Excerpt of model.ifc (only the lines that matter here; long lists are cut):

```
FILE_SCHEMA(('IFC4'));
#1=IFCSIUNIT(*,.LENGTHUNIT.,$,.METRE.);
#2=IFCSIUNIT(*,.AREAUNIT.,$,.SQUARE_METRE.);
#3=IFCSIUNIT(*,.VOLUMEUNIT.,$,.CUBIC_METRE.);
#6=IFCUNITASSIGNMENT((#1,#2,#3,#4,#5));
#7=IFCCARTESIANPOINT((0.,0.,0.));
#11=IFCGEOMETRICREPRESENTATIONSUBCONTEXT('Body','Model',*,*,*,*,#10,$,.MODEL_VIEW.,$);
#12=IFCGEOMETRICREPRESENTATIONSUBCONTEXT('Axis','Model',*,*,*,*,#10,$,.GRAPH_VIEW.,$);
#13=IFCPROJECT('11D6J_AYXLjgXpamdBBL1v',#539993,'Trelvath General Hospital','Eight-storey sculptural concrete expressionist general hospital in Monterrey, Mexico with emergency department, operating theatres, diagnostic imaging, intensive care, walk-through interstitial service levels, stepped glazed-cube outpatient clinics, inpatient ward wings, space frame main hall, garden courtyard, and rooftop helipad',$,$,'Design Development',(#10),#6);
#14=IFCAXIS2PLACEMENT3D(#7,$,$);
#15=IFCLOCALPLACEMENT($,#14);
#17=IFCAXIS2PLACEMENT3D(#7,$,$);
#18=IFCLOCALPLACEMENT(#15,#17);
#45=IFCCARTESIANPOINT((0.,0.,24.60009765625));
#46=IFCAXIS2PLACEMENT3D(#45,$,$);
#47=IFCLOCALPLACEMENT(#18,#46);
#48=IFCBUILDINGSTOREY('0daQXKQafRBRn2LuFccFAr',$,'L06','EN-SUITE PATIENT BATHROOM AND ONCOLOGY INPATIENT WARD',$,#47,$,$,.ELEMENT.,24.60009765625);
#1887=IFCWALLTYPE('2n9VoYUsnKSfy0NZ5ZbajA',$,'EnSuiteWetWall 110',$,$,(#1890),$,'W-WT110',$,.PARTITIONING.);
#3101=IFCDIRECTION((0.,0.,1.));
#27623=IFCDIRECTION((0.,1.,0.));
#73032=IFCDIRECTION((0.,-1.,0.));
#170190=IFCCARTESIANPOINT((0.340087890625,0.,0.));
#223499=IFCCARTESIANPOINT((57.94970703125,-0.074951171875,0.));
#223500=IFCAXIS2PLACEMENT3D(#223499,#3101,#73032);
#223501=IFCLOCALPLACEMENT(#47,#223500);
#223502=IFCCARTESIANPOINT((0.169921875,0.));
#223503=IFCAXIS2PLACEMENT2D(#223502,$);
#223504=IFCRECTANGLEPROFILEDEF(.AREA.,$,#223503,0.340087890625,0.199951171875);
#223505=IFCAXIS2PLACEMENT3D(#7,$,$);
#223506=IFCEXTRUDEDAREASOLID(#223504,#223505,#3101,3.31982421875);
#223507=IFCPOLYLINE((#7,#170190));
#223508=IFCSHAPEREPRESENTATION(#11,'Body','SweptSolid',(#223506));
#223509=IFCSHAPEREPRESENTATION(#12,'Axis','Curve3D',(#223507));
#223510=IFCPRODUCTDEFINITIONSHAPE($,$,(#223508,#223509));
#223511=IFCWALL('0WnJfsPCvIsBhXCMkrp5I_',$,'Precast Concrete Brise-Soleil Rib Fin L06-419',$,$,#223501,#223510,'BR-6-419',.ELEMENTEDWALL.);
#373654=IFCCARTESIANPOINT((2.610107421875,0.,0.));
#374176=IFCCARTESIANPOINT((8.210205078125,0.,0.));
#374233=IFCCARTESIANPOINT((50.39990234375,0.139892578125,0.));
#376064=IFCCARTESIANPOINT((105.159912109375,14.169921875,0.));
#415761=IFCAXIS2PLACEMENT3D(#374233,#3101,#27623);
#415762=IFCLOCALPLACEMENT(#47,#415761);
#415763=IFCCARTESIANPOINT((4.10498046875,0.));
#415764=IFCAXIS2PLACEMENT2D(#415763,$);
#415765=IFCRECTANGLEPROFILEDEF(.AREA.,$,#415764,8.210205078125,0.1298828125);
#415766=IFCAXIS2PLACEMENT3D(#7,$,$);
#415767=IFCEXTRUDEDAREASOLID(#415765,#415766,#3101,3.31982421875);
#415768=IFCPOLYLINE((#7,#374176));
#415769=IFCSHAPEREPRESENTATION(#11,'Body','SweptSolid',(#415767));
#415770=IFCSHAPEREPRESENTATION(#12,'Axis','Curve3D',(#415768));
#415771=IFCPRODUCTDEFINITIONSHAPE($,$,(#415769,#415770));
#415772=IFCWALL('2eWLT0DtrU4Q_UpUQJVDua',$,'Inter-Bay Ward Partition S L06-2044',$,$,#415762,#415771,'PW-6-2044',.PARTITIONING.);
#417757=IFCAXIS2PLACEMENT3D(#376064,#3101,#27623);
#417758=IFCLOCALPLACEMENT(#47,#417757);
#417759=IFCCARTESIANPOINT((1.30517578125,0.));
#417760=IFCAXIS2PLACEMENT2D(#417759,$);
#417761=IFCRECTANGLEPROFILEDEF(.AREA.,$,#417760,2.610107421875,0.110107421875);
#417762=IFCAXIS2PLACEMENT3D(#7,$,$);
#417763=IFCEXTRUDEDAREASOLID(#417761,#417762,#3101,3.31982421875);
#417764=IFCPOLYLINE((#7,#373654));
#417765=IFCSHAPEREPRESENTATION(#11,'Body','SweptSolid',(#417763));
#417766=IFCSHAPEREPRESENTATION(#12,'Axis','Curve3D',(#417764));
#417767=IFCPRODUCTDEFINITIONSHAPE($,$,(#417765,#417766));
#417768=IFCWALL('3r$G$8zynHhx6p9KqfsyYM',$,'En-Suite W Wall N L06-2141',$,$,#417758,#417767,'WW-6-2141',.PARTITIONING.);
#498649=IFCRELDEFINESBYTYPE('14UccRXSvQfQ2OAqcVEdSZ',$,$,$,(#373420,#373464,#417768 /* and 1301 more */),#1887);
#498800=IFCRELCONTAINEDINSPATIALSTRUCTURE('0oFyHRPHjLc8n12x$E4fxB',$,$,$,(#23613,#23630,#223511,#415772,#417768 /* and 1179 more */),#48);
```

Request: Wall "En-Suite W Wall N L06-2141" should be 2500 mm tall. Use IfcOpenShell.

```python
import ifcopenshell
import ifcopenshell.geom
import ifcopenshell.util.representation
import ifcopenshell.util.shape

model = ifcopenshell.open("model.ifc")
settings = ifcopenshell.geom.settings()


def volume(element):
    """Net volume in cubic metres, openings subtracted."""
    shape = ifcopenshell.geom.create_shape(settings, element)
    return ifcopenshell.util.shape.get_volume(shape.geometry)


wall = model.by_guid("3r$G$8zynHhx6p9KqfsyYM")
before = volume(wall)

body = ifcopenshell.util.representation.get_representation(wall, "Model", "Body")
solid = body.Items[0]
old_height = solid.Depth
solid.Depth = 2.5
after = volume(wall)

print(f"height {old_height:g} -> {solid.Depth:g}, volume {before:.3f} -> {after:.3f} m3")

model.write("model_rev.ifc")
```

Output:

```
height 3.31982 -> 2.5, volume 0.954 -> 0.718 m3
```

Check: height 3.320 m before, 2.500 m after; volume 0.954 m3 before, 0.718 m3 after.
